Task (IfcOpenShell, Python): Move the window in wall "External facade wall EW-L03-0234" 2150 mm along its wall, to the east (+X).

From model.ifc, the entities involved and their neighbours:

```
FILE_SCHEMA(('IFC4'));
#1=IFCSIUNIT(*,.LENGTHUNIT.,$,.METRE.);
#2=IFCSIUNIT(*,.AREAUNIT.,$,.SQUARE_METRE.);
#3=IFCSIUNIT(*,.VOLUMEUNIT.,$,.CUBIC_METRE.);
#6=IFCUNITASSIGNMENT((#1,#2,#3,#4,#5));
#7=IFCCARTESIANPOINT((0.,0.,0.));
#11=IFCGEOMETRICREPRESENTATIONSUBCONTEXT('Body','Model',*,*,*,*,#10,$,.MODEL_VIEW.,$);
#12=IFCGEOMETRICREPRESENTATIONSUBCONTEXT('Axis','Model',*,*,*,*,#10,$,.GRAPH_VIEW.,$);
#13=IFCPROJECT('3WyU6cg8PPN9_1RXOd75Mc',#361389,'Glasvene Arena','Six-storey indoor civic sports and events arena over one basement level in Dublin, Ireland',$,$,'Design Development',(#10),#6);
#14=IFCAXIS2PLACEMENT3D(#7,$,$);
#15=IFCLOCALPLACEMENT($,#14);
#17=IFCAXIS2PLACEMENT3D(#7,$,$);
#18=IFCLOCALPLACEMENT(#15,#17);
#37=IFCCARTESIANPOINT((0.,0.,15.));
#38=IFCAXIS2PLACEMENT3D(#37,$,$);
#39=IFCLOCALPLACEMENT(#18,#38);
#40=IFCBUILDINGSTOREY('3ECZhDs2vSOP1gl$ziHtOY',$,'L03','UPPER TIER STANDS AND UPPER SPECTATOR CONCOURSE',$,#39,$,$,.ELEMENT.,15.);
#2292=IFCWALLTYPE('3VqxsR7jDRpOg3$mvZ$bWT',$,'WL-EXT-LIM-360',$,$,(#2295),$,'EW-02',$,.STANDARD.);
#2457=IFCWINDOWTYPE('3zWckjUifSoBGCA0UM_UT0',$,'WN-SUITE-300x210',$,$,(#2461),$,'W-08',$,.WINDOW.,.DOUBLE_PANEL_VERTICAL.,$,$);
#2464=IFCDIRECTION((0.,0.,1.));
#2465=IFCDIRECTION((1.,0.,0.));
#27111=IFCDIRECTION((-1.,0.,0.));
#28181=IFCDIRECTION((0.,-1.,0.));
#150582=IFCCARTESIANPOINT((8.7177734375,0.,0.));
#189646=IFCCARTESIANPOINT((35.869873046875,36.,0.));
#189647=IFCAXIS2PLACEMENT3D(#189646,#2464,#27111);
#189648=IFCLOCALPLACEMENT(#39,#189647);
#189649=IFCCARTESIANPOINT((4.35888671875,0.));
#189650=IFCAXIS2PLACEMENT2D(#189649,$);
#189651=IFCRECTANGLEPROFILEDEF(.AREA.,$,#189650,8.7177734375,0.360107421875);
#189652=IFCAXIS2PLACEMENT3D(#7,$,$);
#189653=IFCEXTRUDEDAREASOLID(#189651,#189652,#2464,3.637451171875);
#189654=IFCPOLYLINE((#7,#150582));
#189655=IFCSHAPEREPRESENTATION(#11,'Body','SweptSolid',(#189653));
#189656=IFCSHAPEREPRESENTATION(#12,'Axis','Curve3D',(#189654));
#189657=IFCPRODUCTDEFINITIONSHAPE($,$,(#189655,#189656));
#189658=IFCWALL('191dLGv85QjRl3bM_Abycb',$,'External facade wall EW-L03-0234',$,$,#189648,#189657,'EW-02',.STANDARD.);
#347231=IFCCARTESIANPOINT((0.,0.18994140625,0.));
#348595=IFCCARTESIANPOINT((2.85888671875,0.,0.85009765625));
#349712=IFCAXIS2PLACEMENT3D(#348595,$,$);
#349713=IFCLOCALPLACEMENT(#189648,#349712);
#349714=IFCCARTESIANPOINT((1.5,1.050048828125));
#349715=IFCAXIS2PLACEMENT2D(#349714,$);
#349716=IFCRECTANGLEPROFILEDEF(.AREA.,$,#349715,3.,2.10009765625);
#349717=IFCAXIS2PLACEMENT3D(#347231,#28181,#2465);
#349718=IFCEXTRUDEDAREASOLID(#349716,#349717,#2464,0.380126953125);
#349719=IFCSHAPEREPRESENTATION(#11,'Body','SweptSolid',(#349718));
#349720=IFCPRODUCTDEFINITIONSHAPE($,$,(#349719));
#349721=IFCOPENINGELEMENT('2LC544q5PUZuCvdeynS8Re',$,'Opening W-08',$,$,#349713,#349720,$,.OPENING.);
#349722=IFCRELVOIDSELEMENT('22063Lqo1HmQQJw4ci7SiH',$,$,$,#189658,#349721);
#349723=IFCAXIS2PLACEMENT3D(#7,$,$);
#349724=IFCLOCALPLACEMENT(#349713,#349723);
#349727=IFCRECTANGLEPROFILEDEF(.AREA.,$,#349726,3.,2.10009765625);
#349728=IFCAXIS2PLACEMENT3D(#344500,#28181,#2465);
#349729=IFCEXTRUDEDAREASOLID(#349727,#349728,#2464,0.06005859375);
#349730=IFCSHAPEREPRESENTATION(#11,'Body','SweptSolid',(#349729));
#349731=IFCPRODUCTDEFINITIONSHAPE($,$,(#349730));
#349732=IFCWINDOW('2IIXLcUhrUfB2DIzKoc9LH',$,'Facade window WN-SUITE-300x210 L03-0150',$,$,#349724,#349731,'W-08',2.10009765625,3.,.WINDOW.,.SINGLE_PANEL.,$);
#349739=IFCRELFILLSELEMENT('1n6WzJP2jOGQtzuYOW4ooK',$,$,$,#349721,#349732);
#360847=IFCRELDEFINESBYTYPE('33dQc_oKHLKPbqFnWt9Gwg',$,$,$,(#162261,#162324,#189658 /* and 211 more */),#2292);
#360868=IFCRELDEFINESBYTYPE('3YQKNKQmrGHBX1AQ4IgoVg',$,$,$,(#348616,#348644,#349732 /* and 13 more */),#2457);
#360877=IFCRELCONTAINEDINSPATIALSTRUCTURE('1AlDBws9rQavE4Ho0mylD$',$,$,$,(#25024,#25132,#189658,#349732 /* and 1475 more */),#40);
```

```python
import ifcopenshell
import ifcopenshell.api.geometry
import ifcopenshell.util.placement
import ifcopenshell.util.unit

model = ifcopenshell.open("model.ifc")
unit_scale = ifcopenshell.util.unit.calculate_unit_scale(model)

window = model.by_guid("2IIXLcUhrUfB2DIzKoc9LH")
opening = window.FillsVoids[0].RelatingOpeningElement
wall = opening.VoidsElements[0].RelatingBuildingElement

wall_matrix = ifcopenshell.util.placement.get_local_placement(wall.ObjectPlacement)
shift = wall_matrix[:3, 0] * -2.15 / unit_scale
before = ifcopenshell.util.placement.get_local_placement(window.ObjectPlacement)[:3, 3].copy()

# The window is placed relative to its opening, so it follows when the opening moves.
matrix = ifcopenshell.util.placement.get_local_placement(opening.ObjectPlacement)
matrix[:3, 3] += shift
ifcopenshell.api.geometry.edit_object_placement(
    model, product=opening, matrix=matrix, is_si=False, should_transform_children=True
)

after = ifcopenshell.util.placement.get_local_placement(window.ObjectPlacement)[:3, 3]
print("window moved by", (after - before).round(3) + 0.0)

model.write("model_updated.ifc")
```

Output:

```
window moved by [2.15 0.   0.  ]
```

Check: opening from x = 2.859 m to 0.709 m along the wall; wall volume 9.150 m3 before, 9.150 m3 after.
